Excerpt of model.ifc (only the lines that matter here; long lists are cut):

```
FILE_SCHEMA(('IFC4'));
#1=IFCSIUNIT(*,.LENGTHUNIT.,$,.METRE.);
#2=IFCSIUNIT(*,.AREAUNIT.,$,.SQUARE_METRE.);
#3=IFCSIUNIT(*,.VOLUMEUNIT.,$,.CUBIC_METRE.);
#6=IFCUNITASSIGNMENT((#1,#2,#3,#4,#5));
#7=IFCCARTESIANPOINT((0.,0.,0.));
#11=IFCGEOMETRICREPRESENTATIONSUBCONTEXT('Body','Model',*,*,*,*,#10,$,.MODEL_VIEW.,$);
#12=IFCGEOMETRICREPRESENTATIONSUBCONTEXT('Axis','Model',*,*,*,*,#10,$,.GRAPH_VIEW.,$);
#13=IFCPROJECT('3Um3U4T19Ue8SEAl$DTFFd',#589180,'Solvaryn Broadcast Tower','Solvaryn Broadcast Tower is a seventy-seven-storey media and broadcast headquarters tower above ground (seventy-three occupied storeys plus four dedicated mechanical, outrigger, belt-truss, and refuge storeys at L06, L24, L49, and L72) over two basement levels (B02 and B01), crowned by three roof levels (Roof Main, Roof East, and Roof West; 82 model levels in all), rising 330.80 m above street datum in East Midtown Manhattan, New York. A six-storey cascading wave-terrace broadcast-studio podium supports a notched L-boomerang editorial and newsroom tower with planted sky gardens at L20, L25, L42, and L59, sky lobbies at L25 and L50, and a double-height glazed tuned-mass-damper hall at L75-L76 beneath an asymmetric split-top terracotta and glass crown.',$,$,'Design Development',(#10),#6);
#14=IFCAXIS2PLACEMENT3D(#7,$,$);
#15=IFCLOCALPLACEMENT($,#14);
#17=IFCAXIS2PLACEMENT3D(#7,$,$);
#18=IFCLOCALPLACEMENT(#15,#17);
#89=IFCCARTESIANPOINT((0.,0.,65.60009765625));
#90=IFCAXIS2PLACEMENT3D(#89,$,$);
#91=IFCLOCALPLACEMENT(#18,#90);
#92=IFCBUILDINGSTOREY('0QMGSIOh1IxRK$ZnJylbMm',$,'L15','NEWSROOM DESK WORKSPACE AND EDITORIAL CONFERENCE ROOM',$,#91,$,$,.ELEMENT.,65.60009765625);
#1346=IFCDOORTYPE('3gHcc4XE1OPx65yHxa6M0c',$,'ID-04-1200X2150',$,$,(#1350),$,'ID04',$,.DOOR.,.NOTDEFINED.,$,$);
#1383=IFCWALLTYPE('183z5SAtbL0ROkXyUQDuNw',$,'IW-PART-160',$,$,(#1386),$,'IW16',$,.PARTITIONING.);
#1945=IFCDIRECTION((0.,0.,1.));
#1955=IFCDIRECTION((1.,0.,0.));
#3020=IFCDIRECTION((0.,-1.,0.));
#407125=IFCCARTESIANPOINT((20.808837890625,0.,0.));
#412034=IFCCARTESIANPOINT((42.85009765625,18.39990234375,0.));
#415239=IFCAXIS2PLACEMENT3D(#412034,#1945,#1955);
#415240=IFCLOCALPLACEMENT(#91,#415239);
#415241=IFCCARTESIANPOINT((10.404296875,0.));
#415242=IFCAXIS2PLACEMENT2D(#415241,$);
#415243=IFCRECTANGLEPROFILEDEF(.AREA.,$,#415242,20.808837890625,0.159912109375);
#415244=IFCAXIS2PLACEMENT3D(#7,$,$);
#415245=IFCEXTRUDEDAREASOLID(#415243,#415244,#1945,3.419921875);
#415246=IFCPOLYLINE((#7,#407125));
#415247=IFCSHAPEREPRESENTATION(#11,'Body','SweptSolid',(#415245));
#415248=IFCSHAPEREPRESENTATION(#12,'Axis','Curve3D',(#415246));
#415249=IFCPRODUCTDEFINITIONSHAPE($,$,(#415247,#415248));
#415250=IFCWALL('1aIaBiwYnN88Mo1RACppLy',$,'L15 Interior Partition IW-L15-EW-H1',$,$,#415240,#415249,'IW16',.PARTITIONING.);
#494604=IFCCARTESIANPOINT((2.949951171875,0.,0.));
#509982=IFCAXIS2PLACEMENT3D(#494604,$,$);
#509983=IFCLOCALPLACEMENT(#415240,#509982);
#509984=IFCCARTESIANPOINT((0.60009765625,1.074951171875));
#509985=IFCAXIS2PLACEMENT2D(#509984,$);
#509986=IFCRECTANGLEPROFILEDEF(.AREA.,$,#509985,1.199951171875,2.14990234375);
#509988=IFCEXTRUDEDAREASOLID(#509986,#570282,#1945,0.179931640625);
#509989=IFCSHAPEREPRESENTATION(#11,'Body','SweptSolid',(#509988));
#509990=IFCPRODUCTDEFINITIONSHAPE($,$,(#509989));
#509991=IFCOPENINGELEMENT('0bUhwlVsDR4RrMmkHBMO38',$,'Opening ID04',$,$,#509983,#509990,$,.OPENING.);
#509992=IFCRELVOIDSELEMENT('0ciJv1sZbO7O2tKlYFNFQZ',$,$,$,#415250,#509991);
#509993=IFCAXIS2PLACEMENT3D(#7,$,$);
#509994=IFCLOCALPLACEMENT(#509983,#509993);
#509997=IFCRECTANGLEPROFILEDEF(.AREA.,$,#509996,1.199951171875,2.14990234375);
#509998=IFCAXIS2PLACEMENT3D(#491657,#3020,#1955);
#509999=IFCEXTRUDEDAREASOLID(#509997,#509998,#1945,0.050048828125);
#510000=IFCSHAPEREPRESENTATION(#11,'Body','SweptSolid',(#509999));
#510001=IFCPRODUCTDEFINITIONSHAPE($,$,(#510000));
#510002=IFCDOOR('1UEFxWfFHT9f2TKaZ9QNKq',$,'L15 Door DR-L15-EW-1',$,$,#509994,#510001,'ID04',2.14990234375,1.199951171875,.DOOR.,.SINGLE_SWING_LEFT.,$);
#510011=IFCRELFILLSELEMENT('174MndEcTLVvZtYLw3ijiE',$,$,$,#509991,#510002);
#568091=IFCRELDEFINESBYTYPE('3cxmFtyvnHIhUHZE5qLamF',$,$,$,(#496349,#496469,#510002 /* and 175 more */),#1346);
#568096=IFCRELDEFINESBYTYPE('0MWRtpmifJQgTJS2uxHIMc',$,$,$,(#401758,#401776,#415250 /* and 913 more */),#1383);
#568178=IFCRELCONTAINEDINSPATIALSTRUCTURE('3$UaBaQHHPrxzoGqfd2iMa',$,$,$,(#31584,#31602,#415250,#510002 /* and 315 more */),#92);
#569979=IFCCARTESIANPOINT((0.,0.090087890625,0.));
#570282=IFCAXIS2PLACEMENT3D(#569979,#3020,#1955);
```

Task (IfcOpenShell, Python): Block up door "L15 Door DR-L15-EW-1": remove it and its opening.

```python
import ifcopenshell
import ifcopenshell.api.feature
import ifcopenshell.api.root
import ifcopenshell.geom
import ifcopenshell.util.shape

model = ifcopenshell.open("model.ifc")
settings = ifcopenshell.geom.settings()


def volume(element):
    """Net volume in cubic metres, openings subtracted."""
    shape = ifcopenshell.geom.create_shape(settings, element)
    return ifcopenshell.util.shape.get_volume(shape.geometry)


door = model.by_guid("1UEFxWfFHT9f2TKaZ9QNKq")
opening = door.FillsVoids[0].RelatingOpeningElement
wall = opening.VoidsElements[0].RelatingBuildingElement
before = volume(wall)

ifcopenshell.api.root.remove_product(model, product=door)
ifcopenshell.api.feature.remove_feature(model, feature=opening)

after = volume(wall)

print(f"wall volume {before:.3f} -> {after:.3f} m3")

model.write("model_updated.ifc")
```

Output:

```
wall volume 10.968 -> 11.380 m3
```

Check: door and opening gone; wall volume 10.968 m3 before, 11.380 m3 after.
